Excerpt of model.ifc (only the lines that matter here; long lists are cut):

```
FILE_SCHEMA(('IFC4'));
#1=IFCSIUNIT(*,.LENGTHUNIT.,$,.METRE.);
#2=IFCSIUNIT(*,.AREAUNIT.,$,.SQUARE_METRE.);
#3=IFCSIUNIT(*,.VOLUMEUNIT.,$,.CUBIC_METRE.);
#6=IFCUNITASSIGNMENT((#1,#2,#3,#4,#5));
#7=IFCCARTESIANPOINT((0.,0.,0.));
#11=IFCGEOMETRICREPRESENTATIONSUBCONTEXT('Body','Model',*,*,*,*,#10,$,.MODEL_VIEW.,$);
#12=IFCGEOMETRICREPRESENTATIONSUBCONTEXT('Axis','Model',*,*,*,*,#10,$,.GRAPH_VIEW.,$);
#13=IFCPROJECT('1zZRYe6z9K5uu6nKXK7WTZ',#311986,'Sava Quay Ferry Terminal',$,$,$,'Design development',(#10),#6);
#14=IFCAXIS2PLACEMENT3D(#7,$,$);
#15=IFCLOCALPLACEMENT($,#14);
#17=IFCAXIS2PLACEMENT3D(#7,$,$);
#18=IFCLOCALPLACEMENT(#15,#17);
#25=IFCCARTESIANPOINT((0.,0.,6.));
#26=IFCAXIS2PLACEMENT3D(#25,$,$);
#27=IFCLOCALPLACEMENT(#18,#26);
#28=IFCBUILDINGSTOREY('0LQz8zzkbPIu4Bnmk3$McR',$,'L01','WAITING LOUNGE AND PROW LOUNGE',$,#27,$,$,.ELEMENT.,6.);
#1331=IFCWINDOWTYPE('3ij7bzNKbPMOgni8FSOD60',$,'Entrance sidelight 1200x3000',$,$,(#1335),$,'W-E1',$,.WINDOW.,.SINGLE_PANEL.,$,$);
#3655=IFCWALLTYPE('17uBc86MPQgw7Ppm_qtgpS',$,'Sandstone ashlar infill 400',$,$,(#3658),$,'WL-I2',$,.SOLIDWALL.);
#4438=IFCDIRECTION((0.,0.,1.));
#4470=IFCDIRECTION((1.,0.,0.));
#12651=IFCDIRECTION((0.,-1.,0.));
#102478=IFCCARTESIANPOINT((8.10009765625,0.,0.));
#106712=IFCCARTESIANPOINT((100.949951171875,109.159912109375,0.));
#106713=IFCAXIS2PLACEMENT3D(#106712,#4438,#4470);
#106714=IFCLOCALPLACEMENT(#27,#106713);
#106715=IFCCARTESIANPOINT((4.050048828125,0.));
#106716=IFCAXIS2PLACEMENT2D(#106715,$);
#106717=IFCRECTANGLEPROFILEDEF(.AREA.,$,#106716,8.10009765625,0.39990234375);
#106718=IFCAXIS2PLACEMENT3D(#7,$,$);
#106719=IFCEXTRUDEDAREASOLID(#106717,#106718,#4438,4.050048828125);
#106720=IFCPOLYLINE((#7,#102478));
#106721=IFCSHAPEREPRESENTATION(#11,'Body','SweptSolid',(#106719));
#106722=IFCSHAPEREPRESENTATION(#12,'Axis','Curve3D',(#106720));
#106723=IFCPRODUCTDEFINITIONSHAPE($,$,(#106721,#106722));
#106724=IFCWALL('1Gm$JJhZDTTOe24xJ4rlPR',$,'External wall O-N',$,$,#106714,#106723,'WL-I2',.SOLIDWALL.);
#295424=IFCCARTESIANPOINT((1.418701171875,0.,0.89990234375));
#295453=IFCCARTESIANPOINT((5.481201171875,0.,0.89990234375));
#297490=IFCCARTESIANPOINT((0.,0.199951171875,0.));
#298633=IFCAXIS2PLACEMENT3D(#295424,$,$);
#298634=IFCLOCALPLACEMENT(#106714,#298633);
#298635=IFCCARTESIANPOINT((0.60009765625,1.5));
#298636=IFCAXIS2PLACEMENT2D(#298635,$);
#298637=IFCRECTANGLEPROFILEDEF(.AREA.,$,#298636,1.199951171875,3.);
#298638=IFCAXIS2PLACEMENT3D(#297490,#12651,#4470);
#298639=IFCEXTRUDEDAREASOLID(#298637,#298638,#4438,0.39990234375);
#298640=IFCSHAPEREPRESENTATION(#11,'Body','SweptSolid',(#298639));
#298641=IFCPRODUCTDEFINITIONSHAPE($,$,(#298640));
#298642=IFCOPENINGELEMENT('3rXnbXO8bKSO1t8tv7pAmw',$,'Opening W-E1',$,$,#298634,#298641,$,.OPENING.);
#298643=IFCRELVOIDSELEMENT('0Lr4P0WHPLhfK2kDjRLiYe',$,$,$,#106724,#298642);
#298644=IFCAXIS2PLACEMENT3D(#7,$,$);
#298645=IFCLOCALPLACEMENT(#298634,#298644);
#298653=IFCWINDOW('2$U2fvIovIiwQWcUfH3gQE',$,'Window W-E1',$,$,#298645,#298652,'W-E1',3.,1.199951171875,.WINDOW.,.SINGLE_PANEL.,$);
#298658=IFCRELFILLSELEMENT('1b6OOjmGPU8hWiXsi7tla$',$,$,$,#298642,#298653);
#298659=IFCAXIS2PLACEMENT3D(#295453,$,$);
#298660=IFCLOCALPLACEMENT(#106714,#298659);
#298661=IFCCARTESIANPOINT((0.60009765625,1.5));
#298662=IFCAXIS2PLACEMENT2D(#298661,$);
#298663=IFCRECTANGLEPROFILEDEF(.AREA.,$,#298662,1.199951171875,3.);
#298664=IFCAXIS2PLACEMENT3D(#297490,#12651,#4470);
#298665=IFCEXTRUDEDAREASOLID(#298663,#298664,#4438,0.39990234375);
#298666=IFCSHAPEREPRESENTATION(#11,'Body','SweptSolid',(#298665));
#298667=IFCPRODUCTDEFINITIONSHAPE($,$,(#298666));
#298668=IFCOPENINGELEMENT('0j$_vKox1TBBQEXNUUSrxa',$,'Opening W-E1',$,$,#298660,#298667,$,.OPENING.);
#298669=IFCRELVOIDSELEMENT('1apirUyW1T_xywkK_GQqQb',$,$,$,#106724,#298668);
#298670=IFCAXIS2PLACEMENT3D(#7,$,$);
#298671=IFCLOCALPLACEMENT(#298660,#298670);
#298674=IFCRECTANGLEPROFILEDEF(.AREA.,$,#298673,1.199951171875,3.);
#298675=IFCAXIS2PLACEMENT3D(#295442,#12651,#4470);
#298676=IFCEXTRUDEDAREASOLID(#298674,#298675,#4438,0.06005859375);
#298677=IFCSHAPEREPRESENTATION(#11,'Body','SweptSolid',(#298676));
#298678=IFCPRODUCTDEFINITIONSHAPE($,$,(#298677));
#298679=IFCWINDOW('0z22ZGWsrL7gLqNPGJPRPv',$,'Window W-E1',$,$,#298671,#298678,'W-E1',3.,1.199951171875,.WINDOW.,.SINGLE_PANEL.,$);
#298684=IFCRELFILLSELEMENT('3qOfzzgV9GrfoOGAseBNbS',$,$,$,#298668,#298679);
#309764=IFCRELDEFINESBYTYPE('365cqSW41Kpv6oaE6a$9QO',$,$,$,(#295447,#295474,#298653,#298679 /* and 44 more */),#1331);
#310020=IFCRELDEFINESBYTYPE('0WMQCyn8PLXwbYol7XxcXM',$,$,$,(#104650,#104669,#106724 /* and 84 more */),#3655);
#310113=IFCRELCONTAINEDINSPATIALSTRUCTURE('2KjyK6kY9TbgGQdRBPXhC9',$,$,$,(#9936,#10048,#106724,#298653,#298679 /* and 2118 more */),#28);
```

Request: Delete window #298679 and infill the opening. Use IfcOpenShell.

```python
import ifcopenshell
import ifcopenshell.api.feature
import ifcopenshell.api.root
import ifcopenshell.geom
import ifcopenshell.util.shape

model = ifcopenshell.open("model.ifc")
settings = ifcopenshell.geom.settings()


def volume(element):
    """Net volume in cubic metres, openings subtracted."""
    shape = ifcopenshell.geom.create_shape(settings, element)
    return ifcopenshell.util.shape.get_volume(shape.geometry)


window = model.by_guid("0z22ZGWsrL7gLqNPGJPRPv")
opening = window.FillsVoids[0].RelatingOpeningElement
wall = opening.VoidsElements[0].RelatingBuildingElement
before = volume(wall)

ifcopenshell.api.root.remove_product(model, product=window)
ifcopenshell.api.feature.remove_feature(model, feature=opening)

after = volume(wall)

print(f"wall volume {before:.3f} -> {after:.3f} m3")

model.write("model_updated.ifc")
```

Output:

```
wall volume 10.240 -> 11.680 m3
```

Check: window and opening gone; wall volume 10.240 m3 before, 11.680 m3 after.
